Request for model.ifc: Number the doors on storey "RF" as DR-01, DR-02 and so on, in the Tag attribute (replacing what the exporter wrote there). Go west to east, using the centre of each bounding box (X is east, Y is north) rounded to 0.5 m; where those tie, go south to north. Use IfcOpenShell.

First a look at what the model holds.

```python
import ifcopenshell
import ifcopenshell.util.element
import ifcopenshell.util.placement

model = ifcopenshell.open("model.ifc")
print(model.schema)
storey = next(s for s in model.by_type("IfcBuildingStorey") if s.Name == "RF")
doors = [e for e in ifcopenshell.util.element.get_decomposition(storey) if e.is_a("IfcDoor")]
for e in sorted(doors, key=lambda e: e.id()):
    origin = ifcopenshell.util.placement.get_local_placement(e.ObjectPlacement)[:3, 3]
    print(e.id(), e.Tag, e.Name, origin.round(2) + 0.0, sep=" | ")
```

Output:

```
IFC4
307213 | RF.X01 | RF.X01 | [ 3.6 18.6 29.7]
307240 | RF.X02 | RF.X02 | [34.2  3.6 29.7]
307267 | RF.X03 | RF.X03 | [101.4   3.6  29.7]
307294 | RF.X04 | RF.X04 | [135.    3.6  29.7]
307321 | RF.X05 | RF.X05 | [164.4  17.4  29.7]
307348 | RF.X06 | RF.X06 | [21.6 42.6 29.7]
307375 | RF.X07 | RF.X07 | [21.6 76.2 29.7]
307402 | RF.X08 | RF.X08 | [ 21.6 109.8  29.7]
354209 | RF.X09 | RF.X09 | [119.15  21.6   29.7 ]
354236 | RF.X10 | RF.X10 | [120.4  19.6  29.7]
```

```python
import ifcopenshell
import ifcopenshell.geom
import ifcopenshell.util.element
import ifcopenshell.util.shape

model = ifcopenshell.open("model.ifc")
settings = ifcopenshell.geom.settings()
settings.set("use-world-coords", True)


def centre(element):
    shape = ifcopenshell.geom.create_shape(settings, element)
    return ifcopenshell.util.shape.get_bbox_centroid(shape.geometry)


storey = next(s for s in model.by_type("IfcBuildingStorey") if s.Name == "RF")
doors = [e for e in ifcopenshell.util.element.get_decomposition(storey) if e.is_a("IfcDoor")]

# Insertion points can sit at a corner or the storey origin, so sort by the geometry (in metres).
centres = {e: centre(e) for e in doors}
doors.sort(key=lambda e: (round(centres[e][0] / 0.5), centres[e][1]))

for i, e in enumerate(doors, start=1):
    number = f"DR-{i:02d}"
    e.Tag = number
    print(e.id(), number)

model.write("model-out.ifc")
```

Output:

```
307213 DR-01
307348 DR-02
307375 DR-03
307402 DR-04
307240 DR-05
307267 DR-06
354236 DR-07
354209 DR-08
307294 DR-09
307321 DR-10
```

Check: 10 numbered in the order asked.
